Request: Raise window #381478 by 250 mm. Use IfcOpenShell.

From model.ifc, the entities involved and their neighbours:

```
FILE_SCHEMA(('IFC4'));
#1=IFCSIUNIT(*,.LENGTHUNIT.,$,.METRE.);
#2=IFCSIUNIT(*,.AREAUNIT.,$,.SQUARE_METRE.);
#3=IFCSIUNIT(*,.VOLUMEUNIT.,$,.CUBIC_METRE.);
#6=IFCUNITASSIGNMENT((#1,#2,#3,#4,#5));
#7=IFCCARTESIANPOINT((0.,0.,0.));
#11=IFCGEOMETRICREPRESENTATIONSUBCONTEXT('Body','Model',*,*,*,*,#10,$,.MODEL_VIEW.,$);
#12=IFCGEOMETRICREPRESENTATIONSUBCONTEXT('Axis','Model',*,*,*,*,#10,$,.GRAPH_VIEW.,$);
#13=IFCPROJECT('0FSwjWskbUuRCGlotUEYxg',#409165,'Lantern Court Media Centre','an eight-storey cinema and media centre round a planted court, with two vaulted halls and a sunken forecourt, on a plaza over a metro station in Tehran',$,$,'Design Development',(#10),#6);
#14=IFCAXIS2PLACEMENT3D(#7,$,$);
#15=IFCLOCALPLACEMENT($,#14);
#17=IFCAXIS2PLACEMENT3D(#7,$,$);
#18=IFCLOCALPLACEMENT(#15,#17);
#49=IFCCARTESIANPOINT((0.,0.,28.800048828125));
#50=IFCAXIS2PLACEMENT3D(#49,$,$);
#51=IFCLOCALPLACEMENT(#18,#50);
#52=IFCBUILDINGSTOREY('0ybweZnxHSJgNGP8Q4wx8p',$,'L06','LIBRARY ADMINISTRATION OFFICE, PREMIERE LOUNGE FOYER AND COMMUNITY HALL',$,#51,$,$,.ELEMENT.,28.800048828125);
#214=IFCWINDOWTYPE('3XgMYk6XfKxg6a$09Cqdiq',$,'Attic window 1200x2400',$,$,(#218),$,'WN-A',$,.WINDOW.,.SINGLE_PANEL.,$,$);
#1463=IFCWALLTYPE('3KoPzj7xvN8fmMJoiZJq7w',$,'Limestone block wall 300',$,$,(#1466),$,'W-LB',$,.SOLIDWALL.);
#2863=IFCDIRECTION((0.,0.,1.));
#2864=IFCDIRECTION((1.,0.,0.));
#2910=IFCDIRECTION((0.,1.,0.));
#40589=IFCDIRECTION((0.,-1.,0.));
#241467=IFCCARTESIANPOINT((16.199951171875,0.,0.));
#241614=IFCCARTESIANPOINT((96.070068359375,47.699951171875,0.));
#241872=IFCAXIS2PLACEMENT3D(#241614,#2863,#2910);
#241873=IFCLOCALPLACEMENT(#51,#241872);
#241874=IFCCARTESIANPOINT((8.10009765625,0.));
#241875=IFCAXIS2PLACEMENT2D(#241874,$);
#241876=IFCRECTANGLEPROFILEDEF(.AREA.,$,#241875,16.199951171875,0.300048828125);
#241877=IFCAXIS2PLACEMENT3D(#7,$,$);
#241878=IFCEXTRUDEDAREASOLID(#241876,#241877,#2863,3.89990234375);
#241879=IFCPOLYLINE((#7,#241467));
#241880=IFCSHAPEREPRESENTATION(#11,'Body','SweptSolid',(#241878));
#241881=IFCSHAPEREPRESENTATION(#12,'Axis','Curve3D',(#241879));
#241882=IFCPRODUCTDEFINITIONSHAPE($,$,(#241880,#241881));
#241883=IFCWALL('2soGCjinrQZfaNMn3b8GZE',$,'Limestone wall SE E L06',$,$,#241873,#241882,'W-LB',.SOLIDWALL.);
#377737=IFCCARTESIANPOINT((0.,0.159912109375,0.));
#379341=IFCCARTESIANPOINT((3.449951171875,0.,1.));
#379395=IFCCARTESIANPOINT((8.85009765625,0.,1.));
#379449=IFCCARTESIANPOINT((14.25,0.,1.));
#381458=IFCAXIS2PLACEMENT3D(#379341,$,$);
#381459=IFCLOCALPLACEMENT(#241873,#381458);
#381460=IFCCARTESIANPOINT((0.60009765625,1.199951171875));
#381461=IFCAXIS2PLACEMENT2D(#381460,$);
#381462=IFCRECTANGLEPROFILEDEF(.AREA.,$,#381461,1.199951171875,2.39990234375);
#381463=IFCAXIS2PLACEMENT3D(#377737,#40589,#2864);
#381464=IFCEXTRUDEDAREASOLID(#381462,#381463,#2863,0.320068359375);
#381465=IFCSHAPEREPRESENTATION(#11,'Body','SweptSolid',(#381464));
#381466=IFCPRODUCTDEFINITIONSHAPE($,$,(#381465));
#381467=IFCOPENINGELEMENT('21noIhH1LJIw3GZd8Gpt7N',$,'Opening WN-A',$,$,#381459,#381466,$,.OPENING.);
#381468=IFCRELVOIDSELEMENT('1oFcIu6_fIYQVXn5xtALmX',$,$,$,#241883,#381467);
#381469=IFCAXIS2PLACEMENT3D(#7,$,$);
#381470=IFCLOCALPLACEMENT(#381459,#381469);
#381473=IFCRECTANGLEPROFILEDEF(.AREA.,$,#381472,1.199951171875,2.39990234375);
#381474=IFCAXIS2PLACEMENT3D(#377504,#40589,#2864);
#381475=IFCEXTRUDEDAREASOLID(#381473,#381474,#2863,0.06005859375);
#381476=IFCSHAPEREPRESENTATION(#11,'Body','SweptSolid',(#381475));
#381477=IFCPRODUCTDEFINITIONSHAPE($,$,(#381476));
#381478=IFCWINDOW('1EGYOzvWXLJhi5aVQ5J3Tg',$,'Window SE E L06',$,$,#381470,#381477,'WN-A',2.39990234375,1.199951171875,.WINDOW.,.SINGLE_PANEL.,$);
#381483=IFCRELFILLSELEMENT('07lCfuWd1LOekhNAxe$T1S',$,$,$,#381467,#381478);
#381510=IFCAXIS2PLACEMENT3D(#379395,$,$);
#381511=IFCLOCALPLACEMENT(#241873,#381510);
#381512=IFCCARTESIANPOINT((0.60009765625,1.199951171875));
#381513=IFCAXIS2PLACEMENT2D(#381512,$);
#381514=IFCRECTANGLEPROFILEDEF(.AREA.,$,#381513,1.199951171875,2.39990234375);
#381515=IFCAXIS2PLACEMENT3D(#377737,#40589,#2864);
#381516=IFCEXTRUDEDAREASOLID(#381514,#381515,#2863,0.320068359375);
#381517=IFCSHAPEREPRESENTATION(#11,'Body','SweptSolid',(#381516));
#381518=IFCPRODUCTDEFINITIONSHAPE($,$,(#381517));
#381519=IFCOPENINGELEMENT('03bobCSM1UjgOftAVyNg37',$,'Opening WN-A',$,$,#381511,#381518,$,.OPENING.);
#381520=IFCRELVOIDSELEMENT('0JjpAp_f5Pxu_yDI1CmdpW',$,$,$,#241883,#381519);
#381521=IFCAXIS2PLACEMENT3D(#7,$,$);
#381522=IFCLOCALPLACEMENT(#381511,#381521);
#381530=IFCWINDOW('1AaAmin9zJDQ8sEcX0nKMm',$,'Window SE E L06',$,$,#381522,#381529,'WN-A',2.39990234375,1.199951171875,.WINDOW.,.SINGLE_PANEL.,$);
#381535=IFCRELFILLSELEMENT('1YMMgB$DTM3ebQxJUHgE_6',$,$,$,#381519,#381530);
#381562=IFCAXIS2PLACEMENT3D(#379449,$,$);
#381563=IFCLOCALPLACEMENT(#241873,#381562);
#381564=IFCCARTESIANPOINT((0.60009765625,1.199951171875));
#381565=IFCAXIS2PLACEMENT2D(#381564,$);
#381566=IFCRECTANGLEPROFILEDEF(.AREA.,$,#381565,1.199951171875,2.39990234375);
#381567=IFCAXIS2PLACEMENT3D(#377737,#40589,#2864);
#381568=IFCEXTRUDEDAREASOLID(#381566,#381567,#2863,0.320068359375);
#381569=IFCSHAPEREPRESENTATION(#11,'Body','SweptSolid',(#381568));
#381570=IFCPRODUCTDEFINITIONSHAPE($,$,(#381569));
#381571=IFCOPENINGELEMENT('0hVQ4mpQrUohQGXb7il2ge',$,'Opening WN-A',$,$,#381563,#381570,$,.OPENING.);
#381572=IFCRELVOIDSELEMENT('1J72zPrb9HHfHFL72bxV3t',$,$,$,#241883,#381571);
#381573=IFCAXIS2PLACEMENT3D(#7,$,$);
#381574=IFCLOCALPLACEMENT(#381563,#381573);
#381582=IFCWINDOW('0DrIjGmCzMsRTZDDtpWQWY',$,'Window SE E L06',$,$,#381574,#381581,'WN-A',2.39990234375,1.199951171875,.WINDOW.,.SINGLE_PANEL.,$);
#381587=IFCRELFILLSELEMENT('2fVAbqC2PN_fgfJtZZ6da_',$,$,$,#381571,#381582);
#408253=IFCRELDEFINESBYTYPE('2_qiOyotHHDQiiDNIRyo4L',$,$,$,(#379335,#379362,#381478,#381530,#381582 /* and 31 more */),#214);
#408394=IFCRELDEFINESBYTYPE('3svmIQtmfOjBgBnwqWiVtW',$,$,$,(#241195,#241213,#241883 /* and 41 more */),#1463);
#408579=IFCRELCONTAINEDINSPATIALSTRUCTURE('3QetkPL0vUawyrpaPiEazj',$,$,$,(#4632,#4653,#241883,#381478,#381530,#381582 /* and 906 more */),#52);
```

```python
import numpy as np
import ifcopenshell
import ifcopenshell.api.geometry
import ifcopenshell.util.placement
import ifcopenshell.util.unit

model = ifcopenshell.open("model.ifc")
unit_scale = ifcopenshell.util.unit.calculate_unit_scale(model)

window = model.by_id(381478)
opening = window.FillsVoids[0].RelatingOpeningElement
dz = 0.25 / unit_scale

shift = np.array([0.0, 0.0, dz])
# The window is placed relative to its opening, so it follows when the opening moves.
matrix = ifcopenshell.util.placement.get_local_placement(opening.ObjectPlacement)
matrix[:3, 3] += shift
ifcopenshell.api.geometry.edit_object_placement(
    model, product=opening, matrix=matrix, is_si=False, should_transform_children=True
)

print(f"moved by {dz * unit_scale:+.3f} m")

model.write("model-out.ifc")
```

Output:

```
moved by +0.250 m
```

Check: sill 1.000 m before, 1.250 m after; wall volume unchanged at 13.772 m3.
